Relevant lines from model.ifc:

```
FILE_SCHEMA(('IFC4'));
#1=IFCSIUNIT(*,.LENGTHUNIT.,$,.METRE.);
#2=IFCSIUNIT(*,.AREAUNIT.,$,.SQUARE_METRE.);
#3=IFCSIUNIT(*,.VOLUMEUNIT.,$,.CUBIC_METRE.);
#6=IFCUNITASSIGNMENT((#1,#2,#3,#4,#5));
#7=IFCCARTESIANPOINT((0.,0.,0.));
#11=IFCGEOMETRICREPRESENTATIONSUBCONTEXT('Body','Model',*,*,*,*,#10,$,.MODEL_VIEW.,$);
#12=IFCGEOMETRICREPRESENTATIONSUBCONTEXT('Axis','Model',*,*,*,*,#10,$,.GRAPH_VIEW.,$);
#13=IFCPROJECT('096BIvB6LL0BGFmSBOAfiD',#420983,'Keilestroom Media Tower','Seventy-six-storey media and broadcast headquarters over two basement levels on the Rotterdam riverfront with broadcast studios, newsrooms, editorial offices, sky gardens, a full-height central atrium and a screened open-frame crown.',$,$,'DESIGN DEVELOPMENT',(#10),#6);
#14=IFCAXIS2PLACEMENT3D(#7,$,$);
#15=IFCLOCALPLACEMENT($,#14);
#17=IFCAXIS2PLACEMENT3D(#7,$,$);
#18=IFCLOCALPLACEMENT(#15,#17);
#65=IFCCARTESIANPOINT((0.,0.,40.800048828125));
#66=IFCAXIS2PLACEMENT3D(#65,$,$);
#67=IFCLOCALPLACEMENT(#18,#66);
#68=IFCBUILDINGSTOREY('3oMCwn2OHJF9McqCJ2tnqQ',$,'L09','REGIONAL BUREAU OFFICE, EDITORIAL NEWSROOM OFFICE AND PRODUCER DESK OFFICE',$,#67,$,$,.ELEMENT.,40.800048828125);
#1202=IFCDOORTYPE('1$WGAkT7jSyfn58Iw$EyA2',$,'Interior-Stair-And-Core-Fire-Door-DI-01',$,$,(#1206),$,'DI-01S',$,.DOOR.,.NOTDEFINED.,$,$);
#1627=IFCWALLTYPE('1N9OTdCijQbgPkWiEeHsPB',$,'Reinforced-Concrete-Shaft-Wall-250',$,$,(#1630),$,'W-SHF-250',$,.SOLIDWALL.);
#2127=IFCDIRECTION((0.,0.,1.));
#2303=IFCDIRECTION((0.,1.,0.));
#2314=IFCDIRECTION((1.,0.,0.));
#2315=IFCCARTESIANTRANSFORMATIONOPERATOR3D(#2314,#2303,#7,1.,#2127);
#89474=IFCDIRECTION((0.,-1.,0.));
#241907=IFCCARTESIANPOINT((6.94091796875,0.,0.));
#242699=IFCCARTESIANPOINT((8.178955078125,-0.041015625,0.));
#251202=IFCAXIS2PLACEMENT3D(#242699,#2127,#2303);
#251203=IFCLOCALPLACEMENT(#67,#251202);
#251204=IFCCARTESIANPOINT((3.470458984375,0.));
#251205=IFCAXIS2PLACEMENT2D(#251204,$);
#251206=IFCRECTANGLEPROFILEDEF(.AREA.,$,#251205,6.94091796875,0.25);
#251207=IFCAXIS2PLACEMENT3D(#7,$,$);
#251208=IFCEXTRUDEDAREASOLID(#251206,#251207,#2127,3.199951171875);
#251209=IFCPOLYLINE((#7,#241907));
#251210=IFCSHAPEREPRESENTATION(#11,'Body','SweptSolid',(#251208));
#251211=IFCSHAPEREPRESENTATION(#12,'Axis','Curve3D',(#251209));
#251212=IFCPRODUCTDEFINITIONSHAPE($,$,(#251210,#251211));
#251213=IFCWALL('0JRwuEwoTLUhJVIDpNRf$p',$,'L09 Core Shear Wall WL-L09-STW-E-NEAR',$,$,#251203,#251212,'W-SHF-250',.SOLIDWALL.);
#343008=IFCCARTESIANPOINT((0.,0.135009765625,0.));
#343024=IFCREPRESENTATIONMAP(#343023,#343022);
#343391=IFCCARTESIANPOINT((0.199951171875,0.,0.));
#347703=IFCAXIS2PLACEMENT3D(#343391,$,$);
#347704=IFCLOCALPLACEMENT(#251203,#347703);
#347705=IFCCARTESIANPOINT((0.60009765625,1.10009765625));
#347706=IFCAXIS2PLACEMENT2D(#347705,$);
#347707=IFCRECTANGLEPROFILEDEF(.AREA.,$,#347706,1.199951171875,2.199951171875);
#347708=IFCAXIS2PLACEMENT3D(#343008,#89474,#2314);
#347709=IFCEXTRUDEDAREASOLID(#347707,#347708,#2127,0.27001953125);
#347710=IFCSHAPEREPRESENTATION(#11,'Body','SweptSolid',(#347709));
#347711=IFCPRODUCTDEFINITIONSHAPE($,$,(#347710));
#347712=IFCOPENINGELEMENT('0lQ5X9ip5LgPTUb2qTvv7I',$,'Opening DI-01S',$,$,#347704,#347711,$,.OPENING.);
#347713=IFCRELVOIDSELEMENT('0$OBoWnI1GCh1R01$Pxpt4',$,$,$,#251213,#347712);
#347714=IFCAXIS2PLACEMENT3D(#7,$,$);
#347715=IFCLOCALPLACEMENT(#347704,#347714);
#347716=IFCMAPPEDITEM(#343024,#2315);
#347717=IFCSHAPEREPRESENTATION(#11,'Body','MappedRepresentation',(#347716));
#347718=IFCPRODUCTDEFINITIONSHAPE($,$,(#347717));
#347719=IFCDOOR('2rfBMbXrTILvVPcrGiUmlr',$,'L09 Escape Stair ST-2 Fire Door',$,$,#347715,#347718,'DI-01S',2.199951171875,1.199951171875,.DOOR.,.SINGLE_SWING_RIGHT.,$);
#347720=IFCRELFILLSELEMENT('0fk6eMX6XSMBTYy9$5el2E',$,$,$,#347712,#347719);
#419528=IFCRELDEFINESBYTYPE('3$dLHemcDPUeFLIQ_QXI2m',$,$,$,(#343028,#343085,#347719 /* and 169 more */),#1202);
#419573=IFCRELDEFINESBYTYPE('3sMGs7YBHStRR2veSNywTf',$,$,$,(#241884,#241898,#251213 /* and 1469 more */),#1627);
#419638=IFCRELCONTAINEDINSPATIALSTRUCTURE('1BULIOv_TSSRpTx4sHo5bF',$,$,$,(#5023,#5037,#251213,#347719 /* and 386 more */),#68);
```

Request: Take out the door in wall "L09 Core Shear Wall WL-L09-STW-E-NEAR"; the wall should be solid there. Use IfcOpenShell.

```python
import ifcopenshell
import ifcopenshell.api.feature
import ifcopenshell.api.root
import ifcopenshell.geom
import ifcopenshell.util.shape

model = ifcopenshell.open("model.ifc")
settings = ifcopenshell.geom.settings()


def volume(element):
    """Net volume in cubic metres, openings subtracted."""
    shape = ifcopenshell.geom.create_shape(settings, element)
    return ifcopenshell.util.shape.get_volume(shape.geometry)


door = model.by_guid("2rfBMbXrTILvVPcrGiUmlr")
opening = door.FillsVoids[0].RelatingOpeningElement
wall = opening.VoidsElements[0].RelatingBuildingElement
before = volume(wall)

ifcopenshell.api.root.remove_product(model, product=door)
ifcopenshell.api.feature.remove_feature(model, feature=opening)

after = volume(wall)

print(f"wall volume {before:.3f} -> {after:.3f} m3")

model.write("model_updated.ifc")
```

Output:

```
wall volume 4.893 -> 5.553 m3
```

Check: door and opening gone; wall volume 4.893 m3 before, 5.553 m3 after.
